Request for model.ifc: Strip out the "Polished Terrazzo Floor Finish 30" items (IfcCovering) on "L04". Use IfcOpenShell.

First a look at what the model holds.

```python
import ifcopenshell
import ifcopenshell.util.element

model = ifcopenshell.open("model.ifc")
print(model.schema)
storey = next(s for s in model.by_type("IfcBuildingStorey") if s.Name == "L04")
coverings = [e for e in ifcopenshell.util.element.get_decomposition(storey) if e.is_a("IfcCovering")]
seen = {}
for e in coverings:
    element_type = ifcopenshell.util.element.get_type(e)
    name = element_type.Name if element_type not in (None, e) else None
    seen[name] = seen.get(name, 0) + 1
for name, count in sorted(seen.items(), key=str):
    print(count, "x", name)
```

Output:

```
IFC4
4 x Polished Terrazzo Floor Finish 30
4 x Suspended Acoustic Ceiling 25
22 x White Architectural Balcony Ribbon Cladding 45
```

```python
import ifcopenshell
import ifcopenshell.api.root
import ifcopenshell.util.element

model = ifcopenshell.open("model.ifc")

storey = next(s for s in model.by_type("IfcBuildingStorey") if s.Name == "L04")
coverings = [e for e in ifcopenshell.util.element.get_decomposition(storey) if e.is_a("IfcCovering")]
targets = [e for e in coverings if (t := ifcopenshell.util.element.get_type(e)) not in (None, e) and t.Name == "Polished Terrazzo Floor Finish 30"]

for e in targets:
    ifcopenshell.api.root.remove_product(model, product=e)
print(len(targets), "removed")

model.write("model_updated.ifc")
```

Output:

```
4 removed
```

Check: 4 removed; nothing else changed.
